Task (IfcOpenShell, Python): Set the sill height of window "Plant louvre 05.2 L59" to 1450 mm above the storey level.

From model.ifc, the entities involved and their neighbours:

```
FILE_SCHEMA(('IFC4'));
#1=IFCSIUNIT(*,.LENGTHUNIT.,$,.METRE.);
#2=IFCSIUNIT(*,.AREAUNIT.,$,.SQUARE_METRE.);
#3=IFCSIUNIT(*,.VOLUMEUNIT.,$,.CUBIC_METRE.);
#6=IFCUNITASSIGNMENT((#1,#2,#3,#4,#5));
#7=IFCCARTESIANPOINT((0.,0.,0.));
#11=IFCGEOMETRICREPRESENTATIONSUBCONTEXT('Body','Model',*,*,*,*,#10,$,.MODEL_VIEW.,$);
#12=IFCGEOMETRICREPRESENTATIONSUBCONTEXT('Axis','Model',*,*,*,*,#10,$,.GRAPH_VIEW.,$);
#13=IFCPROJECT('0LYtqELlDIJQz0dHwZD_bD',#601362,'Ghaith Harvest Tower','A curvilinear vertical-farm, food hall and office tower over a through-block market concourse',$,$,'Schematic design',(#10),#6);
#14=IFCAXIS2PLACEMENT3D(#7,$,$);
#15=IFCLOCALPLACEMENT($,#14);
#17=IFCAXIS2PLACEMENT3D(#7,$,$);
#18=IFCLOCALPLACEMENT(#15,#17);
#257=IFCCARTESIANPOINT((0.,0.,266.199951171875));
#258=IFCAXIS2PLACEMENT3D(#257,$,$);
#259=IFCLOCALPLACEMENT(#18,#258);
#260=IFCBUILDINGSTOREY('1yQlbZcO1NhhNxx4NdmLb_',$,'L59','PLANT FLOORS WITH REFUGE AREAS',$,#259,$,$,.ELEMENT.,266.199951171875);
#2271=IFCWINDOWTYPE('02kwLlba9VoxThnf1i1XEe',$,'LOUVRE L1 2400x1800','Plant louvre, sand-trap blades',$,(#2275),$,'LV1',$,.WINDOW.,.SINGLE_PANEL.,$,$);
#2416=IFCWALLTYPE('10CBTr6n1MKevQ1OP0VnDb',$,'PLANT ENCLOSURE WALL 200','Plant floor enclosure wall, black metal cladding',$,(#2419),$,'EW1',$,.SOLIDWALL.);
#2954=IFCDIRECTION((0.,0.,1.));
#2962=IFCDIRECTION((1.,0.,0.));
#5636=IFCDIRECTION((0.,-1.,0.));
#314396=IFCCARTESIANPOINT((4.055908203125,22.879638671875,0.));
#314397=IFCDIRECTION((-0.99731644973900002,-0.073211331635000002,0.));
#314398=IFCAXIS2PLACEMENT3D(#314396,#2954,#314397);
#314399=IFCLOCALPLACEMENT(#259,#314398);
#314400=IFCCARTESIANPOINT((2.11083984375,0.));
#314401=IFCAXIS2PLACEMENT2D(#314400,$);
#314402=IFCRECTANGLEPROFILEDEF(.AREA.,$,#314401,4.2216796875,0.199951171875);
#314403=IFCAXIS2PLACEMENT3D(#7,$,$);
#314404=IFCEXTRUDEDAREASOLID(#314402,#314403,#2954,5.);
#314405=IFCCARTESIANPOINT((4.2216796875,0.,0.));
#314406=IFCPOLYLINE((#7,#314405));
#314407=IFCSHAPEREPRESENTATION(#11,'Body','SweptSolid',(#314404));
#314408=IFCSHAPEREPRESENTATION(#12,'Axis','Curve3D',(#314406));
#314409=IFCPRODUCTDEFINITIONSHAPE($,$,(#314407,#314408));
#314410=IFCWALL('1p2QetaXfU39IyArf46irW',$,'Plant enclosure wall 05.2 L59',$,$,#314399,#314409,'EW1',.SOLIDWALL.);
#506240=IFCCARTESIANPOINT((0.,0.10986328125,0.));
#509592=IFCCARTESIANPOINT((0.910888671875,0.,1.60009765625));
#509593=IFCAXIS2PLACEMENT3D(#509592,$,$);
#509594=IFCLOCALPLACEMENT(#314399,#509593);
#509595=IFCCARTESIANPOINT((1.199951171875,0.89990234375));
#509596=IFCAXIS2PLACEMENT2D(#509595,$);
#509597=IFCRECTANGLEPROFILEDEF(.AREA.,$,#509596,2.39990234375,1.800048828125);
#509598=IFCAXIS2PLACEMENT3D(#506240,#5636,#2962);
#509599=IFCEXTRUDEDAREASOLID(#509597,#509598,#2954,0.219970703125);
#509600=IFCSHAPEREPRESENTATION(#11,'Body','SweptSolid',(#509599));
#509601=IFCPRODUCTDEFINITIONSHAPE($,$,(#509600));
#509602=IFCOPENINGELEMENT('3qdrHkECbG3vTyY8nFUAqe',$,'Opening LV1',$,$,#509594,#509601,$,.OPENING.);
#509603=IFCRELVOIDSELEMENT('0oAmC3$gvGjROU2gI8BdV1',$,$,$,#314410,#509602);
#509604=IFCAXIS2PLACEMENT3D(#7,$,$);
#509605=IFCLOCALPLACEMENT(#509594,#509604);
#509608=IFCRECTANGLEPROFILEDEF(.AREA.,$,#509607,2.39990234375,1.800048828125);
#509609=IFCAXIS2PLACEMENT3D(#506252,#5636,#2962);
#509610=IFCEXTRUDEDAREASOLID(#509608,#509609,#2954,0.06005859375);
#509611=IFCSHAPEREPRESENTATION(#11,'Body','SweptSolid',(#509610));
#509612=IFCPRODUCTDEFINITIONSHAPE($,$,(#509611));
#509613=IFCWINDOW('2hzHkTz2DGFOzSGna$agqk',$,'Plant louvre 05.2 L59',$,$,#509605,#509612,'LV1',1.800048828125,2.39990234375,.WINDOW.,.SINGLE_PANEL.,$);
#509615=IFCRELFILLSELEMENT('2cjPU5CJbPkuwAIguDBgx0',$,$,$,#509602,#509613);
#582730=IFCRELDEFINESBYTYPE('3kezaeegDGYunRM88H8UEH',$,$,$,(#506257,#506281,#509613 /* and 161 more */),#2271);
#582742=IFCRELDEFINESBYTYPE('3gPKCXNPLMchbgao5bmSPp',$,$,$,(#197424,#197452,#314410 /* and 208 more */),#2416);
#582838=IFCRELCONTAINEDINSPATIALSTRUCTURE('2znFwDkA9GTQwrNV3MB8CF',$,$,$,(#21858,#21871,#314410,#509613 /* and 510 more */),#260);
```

```python
import numpy as np
import ifcopenshell
import ifcopenshell.api.geometry
import ifcopenshell.geom
import ifcopenshell.util.element
import ifcopenshell.util.placement
import ifcopenshell.util.shape
import ifcopenshell.util.unit

model = ifcopenshell.open("model.ifc")
unit_scale = ifcopenshell.util.unit.calculate_unit_scale(model)

window = model.by_id(509613)
opening = window.FillsVoids[0].RelatingOpeningElement
storey = ifcopenshell.util.element.get_container(window, ifc_class="IfcBuildingStorey")
level = ifcopenshell.util.placement.get_local_placement(storey.ObjectPlacement)[2, 3]

# The opening's origin need not be at the sill, so measure its lowest point.
shape = ifcopenshell.geom.create_shape(ifcopenshell.geom.settings(), opening)
bottom = ifcopenshell.util.shape.get_shape_bottom_elevation(shape, shape.geometry) / unit_scale
dz = level + 1.45 - bottom

shift = np.array([0.0, 0.0, dz])
# The window is placed relative to its opening, so it follows when the opening moves.
matrix = ifcopenshell.util.placement.get_local_placement(opening.ObjectPlacement)
matrix[:3, 3] += shift
ifcopenshell.api.geometry.edit_object_placement(
    model, product=opening, matrix=matrix, is_si=False, should_transform_children=True
)

print(f"moved by {dz * unit_scale:+.3f} m")

model.write("model_updated.ifc")
```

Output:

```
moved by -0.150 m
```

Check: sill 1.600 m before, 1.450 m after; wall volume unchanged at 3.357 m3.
